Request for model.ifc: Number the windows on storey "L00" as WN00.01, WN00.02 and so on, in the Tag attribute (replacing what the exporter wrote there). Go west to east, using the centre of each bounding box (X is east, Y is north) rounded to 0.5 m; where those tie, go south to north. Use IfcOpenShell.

First a look at what the model holds.

```python
import ifcopenshell
import ifcopenshell.util.element
import ifcopenshell.util.placement

model = ifcopenshell.open("model.ifc")
print(model.schema)
storey = next(s for s in model.by_type("IfcBuildingStorey") if s.Name == "L00")
windows = [e for e in ifcopenshell.util.element.get_decomposition(storey) if e.is_a("IfcWindow")]
for e in sorted(windows, key=lambda e: e.id()):
    origin = ifcopenshell.util.placement.get_local_placement(e.ObjectPlacement)[:3, 3]
    print(e.id(), e.Tag, e.Name, origin.round(2) + 0.0, sep=" | ")
```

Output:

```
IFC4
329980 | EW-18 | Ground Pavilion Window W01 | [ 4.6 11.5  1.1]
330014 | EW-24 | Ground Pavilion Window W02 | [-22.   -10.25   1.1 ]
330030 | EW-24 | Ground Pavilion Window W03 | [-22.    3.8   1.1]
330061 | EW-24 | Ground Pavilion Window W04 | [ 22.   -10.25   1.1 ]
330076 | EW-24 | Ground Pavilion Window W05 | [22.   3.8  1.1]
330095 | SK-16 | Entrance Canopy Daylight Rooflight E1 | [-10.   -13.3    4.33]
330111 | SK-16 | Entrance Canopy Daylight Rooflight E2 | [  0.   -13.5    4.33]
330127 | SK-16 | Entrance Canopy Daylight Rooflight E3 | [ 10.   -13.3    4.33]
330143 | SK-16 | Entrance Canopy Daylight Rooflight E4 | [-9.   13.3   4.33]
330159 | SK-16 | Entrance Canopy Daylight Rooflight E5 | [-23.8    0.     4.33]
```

```python
import ifcopenshell
import ifcopenshell.geom
import ifcopenshell.util.element
import ifcopenshell.util.shape

model = ifcopenshell.open("model.ifc")
settings = ifcopenshell.geom.settings()
settings.set("use-world-coords", True)


def centre(element):
    shape = ifcopenshell.geom.create_shape(settings, element)
    return ifcopenshell.util.shape.get_bbox_centroid(shape.geometry)


storey = next(s for s in model.by_type("IfcBuildingStorey") if s.Name == "L00")
windows = [e for e in ifcopenshell.util.element.get_decomposition(storey) if e.is_a("IfcWindow")]

# Insertion points can sit at a corner or the storey origin, so sort by the geometry (in metres).
centres = {e: centre(e) for e in windows}
windows.sort(key=lambda e: (round(centres[e][0] / 0.5), centres[e][1]))

for i, e in enumerate(windows, start=1):
    number = f"WN00.{i:02d}"
    e.Tag = number
    print(e.id(), number)

model.write("model_rev.ifc")
```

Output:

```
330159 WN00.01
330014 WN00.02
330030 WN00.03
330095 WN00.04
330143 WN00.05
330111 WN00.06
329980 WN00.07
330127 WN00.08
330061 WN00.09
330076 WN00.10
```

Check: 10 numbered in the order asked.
